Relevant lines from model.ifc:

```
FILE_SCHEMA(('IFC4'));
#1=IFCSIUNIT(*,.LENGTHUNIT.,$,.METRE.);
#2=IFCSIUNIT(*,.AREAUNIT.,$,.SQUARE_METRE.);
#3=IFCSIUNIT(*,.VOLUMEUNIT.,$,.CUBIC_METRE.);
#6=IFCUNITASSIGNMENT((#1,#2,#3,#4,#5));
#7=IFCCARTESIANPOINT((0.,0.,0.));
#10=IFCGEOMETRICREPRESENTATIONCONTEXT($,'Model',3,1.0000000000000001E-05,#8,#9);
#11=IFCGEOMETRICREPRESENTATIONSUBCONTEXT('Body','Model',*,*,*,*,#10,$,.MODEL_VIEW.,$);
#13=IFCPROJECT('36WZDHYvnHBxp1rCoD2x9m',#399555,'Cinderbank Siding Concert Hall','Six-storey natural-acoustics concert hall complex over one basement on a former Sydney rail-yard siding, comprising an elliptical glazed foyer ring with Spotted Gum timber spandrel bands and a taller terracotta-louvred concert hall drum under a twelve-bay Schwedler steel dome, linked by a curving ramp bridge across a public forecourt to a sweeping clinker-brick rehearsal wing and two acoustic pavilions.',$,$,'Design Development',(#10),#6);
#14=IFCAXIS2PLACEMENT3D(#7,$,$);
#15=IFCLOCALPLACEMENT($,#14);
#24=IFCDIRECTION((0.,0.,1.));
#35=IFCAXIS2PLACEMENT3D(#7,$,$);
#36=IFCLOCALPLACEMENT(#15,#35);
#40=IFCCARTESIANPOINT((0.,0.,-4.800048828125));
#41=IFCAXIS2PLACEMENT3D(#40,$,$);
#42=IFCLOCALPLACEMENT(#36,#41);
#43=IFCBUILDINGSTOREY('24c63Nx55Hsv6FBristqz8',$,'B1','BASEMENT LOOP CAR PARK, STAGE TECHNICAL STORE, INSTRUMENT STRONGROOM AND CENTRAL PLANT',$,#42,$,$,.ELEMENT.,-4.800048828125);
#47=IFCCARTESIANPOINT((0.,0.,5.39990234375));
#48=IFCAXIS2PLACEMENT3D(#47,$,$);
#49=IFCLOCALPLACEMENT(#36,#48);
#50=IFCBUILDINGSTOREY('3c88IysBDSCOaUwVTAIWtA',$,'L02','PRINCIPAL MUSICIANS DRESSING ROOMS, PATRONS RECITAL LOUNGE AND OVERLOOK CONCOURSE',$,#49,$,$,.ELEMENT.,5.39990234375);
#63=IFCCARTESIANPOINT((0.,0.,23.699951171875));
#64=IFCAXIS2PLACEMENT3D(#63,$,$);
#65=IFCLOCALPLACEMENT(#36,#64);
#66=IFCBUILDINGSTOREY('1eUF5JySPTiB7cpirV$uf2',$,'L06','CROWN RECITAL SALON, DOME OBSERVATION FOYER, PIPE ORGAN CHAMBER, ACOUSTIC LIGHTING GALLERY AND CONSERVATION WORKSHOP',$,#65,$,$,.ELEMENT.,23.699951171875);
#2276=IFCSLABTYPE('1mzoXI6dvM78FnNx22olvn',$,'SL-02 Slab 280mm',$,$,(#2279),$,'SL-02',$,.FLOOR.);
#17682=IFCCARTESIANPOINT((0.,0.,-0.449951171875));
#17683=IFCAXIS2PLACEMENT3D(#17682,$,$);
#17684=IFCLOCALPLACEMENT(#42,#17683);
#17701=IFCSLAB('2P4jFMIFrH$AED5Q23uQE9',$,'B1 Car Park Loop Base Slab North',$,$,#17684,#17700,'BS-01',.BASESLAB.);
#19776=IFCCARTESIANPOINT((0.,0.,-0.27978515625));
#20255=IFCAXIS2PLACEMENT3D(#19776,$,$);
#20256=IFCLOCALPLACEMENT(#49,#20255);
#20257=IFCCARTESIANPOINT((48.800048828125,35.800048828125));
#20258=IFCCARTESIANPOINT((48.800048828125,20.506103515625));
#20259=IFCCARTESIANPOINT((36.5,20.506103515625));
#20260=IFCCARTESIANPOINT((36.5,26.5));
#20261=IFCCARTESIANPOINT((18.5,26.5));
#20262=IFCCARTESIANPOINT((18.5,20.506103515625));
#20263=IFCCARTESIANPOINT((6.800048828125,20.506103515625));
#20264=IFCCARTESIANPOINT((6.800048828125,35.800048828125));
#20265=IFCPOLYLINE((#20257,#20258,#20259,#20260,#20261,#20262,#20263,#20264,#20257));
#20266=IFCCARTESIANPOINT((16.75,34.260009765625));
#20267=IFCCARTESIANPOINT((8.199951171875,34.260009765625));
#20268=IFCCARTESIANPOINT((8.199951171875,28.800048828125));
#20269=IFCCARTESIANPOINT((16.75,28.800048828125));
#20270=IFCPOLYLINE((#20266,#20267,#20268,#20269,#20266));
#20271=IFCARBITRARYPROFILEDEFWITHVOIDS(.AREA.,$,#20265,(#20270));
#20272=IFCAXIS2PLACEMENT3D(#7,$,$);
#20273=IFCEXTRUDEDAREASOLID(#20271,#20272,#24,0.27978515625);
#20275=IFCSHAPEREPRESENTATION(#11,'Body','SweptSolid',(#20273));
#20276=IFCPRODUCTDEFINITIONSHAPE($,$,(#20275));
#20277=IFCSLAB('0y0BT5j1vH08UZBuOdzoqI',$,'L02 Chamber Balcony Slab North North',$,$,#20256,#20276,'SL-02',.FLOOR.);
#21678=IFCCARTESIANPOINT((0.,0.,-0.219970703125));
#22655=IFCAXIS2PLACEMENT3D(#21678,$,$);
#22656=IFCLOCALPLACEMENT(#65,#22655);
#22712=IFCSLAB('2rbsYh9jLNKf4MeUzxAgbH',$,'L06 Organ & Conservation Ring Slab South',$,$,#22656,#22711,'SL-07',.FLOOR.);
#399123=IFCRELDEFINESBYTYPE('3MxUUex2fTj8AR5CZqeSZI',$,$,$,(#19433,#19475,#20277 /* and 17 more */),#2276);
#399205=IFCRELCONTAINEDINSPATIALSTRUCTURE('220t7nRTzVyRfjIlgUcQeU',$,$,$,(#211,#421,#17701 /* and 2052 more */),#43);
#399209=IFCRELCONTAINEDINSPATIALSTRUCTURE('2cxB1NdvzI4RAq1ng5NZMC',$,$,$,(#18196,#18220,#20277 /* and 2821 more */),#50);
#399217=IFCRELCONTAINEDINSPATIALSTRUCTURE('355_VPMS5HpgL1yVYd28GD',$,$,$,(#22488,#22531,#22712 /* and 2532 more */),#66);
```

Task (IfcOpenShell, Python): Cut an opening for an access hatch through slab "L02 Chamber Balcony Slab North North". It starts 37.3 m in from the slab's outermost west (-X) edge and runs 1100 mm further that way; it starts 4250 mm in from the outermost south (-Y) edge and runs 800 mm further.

```python
import numpy as np
import ifcopenshell
import ifcopenshell.api.feature
import ifcopenshell.api.geometry
import ifcopenshell.api.root
import ifcopenshell.geom
import ifcopenshell.util.placement
import ifcopenshell.util.representation
import ifcopenshell.util.shape
import ifcopenshell.util.unit

model = ifcopenshell.open("model.ifc")
unit_scale = ifcopenshell.util.unit.calculate_unit_scale(model)
settings = ifcopenshell.geom.settings()


def volume(element):
    """Net volume in cubic metres, openings subtracted."""
    shape = ifcopenshell.geom.create_shape(settings, element)
    return ifcopenshell.util.shape.get_volume(shape.geometry)


slab = model.by_guid("0y0BT5j1vH08UZBuOdzoqI")
before = volume(slab)

# Extent in the slab's own axes, in metres. The edges named are its -X and -Y sides.
slab_shape = ifcopenshell.geom.create_shape(settings, slab)
vertices = ifcopenshell.util.shape.get_vertices(slab_shape.geometry)
x_min, y_min, bottom = vertices.min(axis=0)
top = vertices[:, 2].max()

opening = ifcopenshell.api.root.create_entity(model, ifc_class="IfcOpeningElement", name="Access hatch opening", predefined_type="OPENING")
context = ifcopenshell.util.representation.get_context(model, "Model", "Body", "MODEL_VIEW")
width, depth = 1.1, 0.8
outline = [(0.0, 0.0), (width, 0.0), (width, depth), (0.0, depth), (0.0, 0.0)]
# Overshoot both faces by 50 mm so the cut is clean.
shape = ifcopenshell.api.geometry.add_slab_representation(
    model, context=context, depth=top - bottom + 0.1, polyline=outline
)
ifcopenshell.api.geometry.assign_representation(model, product=opening, representation=shape)

matrix = ifcopenshell.util.placement.get_local_placement(slab.ObjectPlacement)
matrix[:, 3] = matrix @ np.append(np.array([x_min + 37.3, y_min + 4.25, bottom - 0.05]) / unit_scale, 1.0)
ifcopenshell.api.geometry.edit_object_placement(model, product=opening, matrix=matrix, is_si=False)
ifcopenshell.api.feature.add_feature(model, feature=opening, element=slab)

after = volume(slab)

print(f"slab volume {before:.3f} -> {after:.3f} m3")

model.write("model_updated.ifc")
```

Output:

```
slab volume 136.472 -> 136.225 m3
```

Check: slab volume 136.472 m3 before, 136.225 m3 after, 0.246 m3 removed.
